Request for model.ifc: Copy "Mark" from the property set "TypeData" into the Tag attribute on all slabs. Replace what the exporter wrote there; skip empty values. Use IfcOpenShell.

First a look at what the model holds.

```python
import ifcopenshell
import ifcopenshell.util.element

model = ifcopenshell.open("model.ifc")
print(model.schema)
slabs = model.by_type("IfcSlab")
print(len(slabs), "slabs")
for e in slabs[:8]:
    source = ifcopenshell.util.element.get_pset(e, "TypeData", "Mark")
    target = e.Tag
    print(e.id(), repr(source), repr(target), sep=" | ")
```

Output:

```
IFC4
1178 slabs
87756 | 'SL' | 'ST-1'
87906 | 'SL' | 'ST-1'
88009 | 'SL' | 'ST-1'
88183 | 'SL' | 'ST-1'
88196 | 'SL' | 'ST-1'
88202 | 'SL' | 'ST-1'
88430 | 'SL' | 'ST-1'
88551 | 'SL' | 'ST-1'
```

```python
import ifcopenshell
import ifcopenshell.util.element

model = ifcopenshell.open("model.ifc")

count = 0
for e in model.by_type("IfcSlab"):
    value = ifcopenshell.util.element.get_pset(e, "TypeData", "Mark")
    current = e.Tag
    if not value or not value.strip() or current == value:
        continue
    e.Tag = value
    count += 1

print(count, "slabs updated")

model.write("model_rev.ifc")
```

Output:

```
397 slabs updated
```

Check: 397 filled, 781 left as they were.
